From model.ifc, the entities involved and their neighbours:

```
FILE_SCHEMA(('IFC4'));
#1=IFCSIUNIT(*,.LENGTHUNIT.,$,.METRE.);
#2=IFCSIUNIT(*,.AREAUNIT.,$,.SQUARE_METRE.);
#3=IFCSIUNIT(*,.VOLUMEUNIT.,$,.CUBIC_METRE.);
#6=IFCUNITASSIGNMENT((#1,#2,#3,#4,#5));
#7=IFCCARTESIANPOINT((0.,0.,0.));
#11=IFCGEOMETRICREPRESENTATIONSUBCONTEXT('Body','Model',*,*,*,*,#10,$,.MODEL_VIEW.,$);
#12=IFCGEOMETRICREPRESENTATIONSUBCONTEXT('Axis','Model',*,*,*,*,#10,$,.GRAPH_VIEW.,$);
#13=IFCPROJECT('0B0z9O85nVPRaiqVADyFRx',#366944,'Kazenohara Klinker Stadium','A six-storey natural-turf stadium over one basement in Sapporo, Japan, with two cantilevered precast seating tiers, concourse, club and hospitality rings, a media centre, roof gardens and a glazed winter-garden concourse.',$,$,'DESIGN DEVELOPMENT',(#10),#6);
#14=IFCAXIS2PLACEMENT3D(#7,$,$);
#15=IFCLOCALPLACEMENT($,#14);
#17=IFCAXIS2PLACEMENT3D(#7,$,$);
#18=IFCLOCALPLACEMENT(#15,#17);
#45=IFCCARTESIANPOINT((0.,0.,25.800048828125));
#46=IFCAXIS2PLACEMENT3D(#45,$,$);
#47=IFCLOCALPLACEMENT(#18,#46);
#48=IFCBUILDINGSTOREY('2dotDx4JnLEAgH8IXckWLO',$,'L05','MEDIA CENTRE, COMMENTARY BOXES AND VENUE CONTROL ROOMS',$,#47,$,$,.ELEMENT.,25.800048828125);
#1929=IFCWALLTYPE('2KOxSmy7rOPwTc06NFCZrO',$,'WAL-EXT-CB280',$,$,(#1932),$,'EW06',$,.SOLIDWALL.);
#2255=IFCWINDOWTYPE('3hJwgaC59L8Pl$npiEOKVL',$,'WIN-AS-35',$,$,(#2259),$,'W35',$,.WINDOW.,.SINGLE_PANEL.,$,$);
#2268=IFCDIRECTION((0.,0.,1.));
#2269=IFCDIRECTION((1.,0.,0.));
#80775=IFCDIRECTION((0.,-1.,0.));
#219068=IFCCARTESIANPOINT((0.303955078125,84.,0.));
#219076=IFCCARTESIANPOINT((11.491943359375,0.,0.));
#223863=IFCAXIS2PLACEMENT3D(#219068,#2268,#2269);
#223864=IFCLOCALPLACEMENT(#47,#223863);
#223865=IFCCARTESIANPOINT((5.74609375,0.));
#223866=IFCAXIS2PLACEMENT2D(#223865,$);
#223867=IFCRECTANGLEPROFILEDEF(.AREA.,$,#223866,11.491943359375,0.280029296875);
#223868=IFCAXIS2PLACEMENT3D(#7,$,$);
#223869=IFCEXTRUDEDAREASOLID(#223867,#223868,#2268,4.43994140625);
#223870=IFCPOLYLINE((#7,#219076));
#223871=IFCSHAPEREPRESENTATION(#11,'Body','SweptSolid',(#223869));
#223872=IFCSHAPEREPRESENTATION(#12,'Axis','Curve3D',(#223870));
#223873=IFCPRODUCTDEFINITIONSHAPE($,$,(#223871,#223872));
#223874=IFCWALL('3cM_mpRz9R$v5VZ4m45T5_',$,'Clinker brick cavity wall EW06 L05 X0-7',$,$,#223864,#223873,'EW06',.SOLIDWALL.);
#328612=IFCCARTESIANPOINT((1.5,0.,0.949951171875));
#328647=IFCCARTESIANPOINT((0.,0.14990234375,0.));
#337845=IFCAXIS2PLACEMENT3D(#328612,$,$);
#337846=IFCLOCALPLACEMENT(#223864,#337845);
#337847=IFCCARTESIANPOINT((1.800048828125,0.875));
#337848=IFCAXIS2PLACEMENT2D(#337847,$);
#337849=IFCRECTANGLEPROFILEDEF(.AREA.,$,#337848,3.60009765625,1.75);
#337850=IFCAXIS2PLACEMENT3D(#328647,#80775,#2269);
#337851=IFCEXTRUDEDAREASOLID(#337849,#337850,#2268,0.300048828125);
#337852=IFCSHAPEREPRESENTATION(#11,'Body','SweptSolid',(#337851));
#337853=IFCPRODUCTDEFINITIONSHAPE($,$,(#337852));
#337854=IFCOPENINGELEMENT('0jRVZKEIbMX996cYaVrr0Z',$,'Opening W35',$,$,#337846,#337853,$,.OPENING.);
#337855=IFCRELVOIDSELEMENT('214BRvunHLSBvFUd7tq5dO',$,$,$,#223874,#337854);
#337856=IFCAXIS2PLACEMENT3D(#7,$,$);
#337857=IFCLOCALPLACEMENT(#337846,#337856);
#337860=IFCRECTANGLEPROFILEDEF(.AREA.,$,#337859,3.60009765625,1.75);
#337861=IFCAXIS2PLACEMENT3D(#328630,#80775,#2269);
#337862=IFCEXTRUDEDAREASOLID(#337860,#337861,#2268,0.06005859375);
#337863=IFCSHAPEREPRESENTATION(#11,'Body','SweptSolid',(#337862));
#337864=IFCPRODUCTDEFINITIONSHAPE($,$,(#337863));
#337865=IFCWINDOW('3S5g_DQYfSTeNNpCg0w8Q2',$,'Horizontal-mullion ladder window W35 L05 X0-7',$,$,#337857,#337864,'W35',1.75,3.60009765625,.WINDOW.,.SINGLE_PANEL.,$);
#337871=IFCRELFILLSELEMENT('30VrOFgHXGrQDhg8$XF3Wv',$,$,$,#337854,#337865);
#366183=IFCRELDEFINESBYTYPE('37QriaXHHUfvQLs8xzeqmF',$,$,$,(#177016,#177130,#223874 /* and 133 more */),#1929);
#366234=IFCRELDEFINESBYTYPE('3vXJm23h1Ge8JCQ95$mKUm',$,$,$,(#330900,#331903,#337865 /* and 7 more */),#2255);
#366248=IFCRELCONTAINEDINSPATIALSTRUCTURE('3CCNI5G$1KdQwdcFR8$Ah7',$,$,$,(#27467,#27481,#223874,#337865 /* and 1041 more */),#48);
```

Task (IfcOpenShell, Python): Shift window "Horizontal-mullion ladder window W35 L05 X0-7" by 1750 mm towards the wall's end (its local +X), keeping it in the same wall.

```python
import ifcopenshell
import ifcopenshell.api.geometry
import ifcopenshell.util.placement
import ifcopenshell.util.unit

model = ifcopenshell.open("model.ifc")
unit_scale = ifcopenshell.util.unit.calculate_unit_scale(model)

window = model.by_id(337865)
opening = window.FillsVoids[0].RelatingOpeningElement
wall = opening.VoidsElements[0].RelatingBuildingElement

wall_matrix = ifcopenshell.util.placement.get_local_placement(wall.ObjectPlacement)
shift = wall_matrix[:3, 0] * 1.75 / unit_scale
before = ifcopenshell.util.placement.get_local_placement(window.ObjectPlacement)[:3, 3].copy()

# The window is placed relative to its opening, so it follows when the opening moves.
matrix = ifcopenshell.util.placement.get_local_placement(opening.ObjectPlacement)
matrix[:3, 3] += shift
ifcopenshell.api.geometry.edit_object_placement(
    model, product=opening, matrix=matrix, is_si=False, should_transform_children=True
)

after = ifcopenshell.util.placement.get_local_placement(window.ObjectPlacement)[:3, 3]
print("window moved by", (after - before).round(3) + 0.0)

model.write("model_v2.ifc")
```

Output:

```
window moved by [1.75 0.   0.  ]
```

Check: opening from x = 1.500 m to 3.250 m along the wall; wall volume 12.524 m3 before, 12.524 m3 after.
